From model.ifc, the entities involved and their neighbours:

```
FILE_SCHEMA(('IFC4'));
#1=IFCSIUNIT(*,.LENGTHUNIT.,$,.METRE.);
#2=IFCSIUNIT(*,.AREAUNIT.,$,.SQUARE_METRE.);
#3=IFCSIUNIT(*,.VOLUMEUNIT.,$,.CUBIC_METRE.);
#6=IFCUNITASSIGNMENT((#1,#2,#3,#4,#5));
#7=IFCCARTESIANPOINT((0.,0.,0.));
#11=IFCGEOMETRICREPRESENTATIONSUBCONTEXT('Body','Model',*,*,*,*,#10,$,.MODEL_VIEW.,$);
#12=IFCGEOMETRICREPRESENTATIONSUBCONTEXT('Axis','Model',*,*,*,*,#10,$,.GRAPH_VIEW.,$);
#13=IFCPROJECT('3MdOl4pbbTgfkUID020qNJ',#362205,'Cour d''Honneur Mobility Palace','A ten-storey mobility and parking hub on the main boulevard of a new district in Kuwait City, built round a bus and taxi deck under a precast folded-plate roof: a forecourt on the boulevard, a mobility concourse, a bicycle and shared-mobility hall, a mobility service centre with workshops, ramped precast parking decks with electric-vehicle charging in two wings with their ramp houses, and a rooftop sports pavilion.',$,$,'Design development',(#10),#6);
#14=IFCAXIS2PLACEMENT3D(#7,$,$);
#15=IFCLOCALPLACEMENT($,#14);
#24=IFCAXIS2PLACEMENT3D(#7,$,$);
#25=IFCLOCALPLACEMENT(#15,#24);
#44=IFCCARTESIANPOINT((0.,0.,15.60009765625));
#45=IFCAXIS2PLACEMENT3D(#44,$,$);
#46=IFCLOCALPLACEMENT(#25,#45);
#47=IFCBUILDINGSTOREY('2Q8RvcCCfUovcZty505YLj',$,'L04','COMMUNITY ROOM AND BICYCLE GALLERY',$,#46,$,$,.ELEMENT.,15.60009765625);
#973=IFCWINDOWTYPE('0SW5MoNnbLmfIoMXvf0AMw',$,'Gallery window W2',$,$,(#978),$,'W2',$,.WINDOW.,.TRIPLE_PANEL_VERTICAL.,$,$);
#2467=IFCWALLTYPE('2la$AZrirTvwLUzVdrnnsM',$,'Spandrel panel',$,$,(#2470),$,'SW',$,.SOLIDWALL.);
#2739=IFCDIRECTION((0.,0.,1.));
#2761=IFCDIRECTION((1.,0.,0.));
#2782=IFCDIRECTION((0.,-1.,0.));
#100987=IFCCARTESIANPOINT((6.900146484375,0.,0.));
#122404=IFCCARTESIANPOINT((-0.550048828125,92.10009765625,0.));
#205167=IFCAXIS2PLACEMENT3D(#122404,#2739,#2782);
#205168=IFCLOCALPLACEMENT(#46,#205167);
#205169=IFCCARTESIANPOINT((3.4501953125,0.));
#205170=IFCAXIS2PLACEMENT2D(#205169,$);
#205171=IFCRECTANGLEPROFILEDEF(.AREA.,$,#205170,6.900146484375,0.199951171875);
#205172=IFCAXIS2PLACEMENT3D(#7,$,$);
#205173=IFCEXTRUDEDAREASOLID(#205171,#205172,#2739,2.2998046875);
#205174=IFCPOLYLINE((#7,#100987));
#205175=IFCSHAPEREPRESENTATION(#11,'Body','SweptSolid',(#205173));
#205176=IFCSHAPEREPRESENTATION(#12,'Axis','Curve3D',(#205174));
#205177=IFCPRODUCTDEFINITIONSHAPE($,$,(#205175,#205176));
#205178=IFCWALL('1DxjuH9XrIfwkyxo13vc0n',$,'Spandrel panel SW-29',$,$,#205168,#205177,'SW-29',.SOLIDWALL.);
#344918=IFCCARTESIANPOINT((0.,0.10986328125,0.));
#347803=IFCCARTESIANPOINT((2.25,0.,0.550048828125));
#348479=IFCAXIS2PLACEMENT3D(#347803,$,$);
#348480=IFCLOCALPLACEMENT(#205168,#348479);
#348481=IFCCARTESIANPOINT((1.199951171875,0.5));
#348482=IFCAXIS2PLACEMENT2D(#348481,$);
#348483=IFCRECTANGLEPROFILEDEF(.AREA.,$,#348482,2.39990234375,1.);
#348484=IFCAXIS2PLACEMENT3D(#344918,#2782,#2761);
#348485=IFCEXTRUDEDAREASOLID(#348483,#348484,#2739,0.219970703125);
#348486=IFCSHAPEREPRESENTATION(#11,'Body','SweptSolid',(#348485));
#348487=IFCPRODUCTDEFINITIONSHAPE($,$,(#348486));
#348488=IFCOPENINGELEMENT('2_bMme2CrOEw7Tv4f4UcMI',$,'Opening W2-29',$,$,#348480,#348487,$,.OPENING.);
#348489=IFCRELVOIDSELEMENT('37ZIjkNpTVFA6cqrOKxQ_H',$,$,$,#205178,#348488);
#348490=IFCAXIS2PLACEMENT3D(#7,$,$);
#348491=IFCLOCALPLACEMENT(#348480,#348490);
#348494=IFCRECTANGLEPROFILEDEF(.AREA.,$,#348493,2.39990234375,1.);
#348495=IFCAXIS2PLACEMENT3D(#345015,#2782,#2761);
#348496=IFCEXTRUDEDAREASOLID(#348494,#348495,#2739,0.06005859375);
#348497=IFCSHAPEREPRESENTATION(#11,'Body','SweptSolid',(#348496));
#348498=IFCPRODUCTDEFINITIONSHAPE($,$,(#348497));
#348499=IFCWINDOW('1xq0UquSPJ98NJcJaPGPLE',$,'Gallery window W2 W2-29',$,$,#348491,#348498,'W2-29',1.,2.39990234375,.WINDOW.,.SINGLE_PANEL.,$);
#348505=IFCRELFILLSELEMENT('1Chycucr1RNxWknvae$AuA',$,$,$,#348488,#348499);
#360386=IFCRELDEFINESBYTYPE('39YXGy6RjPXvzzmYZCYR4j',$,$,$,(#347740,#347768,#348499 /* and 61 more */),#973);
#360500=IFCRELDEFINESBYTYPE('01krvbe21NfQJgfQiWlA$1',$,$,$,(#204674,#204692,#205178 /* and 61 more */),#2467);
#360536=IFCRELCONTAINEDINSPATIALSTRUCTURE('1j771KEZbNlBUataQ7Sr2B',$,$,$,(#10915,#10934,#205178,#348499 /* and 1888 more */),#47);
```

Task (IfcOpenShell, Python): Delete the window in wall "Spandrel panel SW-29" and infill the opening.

```python
import ifcopenshell
import ifcopenshell.api.feature
import ifcopenshell.api.root
import ifcopenshell.geom
import ifcopenshell.util.shape

model = ifcopenshell.open("model.ifc")
settings = ifcopenshell.geom.settings()


def volume(element):
    """Net volume in cubic metres, openings subtracted."""
    shape = ifcopenshell.geom.create_shape(settings, element)
    return ifcopenshell.util.shape.get_volume(shape.geometry)


window = model.by_guid("1xq0UquSPJ98NJcJaPGPLE")
opening = window.FillsVoids[0].RelatingOpeningElement
wall = opening.VoidsElements[0].RelatingBuildingElement
before = volume(wall)

ifcopenshell.api.root.remove_product(model, product=window)
ifcopenshell.api.feature.remove_feature(model, feature=opening)

after = volume(wall)

print(f"wall volume {before:.3f} -> {after:.3f} m3")

model.write("model-out.ifc")
```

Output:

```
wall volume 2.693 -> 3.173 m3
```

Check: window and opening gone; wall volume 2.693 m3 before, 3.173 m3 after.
